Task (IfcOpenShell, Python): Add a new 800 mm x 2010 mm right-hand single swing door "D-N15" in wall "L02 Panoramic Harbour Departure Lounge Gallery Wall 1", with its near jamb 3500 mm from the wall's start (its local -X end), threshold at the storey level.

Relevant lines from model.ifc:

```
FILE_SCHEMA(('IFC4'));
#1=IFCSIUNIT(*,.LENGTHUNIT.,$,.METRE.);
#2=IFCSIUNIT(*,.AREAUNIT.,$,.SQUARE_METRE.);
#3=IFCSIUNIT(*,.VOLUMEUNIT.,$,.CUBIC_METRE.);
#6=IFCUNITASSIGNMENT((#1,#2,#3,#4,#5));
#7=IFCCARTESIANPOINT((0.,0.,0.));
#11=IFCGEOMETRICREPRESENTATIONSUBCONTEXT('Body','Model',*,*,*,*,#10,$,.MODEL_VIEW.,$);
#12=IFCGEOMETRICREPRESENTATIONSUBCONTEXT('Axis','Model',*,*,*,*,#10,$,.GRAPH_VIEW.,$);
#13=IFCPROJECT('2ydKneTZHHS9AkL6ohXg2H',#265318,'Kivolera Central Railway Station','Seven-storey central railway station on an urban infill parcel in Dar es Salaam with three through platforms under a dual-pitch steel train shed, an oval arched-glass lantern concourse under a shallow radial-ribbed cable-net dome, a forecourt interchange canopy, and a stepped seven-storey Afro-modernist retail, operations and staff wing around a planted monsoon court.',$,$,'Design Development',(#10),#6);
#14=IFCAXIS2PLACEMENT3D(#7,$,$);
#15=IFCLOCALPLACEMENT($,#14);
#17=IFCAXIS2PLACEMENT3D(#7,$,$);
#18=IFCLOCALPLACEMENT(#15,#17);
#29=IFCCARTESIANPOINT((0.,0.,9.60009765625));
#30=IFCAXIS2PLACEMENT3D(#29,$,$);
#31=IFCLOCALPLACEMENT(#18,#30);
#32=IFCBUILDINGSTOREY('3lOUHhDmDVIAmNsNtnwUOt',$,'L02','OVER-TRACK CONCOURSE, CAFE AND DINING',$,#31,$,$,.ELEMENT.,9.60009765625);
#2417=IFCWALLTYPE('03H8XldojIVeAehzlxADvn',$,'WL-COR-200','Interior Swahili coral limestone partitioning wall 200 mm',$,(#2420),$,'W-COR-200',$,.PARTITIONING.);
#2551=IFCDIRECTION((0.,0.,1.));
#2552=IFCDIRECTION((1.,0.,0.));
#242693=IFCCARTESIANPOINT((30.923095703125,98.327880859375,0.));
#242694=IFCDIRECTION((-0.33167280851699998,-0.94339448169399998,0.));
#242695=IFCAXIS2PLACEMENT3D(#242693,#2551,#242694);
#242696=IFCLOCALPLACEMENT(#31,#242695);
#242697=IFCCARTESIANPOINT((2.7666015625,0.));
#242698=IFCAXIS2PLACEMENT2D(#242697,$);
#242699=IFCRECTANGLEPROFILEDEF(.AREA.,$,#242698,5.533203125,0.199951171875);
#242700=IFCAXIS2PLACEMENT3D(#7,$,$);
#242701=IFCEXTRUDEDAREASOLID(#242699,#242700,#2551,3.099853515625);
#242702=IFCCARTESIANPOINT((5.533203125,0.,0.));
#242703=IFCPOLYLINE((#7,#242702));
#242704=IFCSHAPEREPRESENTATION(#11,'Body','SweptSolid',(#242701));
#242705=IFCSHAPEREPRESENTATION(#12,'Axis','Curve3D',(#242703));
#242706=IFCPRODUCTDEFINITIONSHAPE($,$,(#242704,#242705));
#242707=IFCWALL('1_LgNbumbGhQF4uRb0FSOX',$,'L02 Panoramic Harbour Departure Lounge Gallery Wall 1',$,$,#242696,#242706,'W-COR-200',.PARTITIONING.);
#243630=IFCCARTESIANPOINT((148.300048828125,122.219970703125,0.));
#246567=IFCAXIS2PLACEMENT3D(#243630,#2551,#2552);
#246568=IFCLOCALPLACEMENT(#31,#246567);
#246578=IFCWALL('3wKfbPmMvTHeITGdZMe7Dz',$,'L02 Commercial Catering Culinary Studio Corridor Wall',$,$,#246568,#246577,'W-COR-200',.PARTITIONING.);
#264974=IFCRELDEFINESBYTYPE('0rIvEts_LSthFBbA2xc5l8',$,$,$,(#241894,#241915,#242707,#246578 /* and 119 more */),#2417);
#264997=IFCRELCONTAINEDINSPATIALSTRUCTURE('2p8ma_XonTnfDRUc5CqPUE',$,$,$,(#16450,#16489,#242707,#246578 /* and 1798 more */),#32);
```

```python
import numpy as np
import ifcopenshell
import ifcopenshell.api.feature
import ifcopenshell.api.geometry
import ifcopenshell.api.root
import ifcopenshell.api.spatial
import ifcopenshell.geom
import ifcopenshell.util.element
import ifcopenshell.util.placement
import ifcopenshell.util.representation
import ifcopenshell.util.shape
import ifcopenshell.util.unit

model = ifcopenshell.open("model.ifc")
unit_scale = ifcopenshell.util.unit.calculate_unit_scale(model)
settings = ifcopenshell.geom.settings()


def volume(element):
    """Net volume in cubic metres, openings subtracted."""
    shape = ifcopenshell.geom.create_shape(settings, element)
    return ifcopenshell.util.shape.get_volume(shape.geometry)


wall = model.by_guid("1_LgNbumbGhQF4uRb0FSOX")
storey = ifcopenshell.util.element.get_container(wall, ifc_class="IfcBuildingStorey")
context = ifcopenshell.util.representation.get_context(model, "Model", "Body", "MODEL_VIEW")
before = volume(wall)

width, height, from_end, sill = 0.8, 2.01, 3.5, 0.0  # metres

# The wall runs along its own X axis, and the end named is its -X end.
wall_shape = ifcopenshell.geom.create_shape(settings, wall)
x, y, z = ifcopenshell.util.shape.get_vertices(wall_shape.geometry).T
start = x.min() + from_end
face, thickness = float(y.min()), float(y.max() - y.min())
wall_matrix = ifcopenshell.util.placement.get_local_placement(wall.ObjectPlacement)
level = ifcopenshell.util.placement.get_local_placement(storey.ObjectPlacement)[2, 3]


def in_wall(x, y):
    """Placement at x, y metres in the wall's axes, at sill height."""
    matrix = wall_matrix.copy()
    matrix[:, 3] = wall_matrix @ np.array([x / unit_scale, y / unit_scale, 0.0, 1.0])
    matrix[2, 3] = level + sill / unit_scale
    return matrix


# Opening: a box that overshoots both wall faces by 50 mm.
opening = ifcopenshell.api.root.create_entity(model, ifc_class="IfcOpeningElement", predefined_type="OPENING")
box = ifcopenshell.api.geometry.add_wall_representation(
    model, context=context, length=width, height=height, thickness=thickness + 0.1
)
ifcopenshell.api.geometry.assign_representation(model, product=opening, representation=box)
ifcopenshell.api.geometry.edit_object_placement(model, product=opening, matrix=in_wall(start, face - 0.05), is_si=False)
ifcopenshell.api.feature.add_feature(model, feature=opening, element=wall)

door = ifcopenshell.api.root.create_entity(model, ifc_class="IfcDoor", name="D-N15", predefined_type="DOOR")
door.OverallWidth, door.OverallHeight = width / unit_scale, height / unit_scale
door.OperationType = "SINGLE_SWING_RIGHT"
body = ifcopenshell.api.geometry.add_door_representation(
    model,
    context=context,
    overall_width=door.OverallWidth,
    overall_height=door.OverallHeight,
    operation_type="SINGLE_SWING_RIGHT",
    lining_properties={"LiningDepth": thickness / unit_scale, "ThresholdDepth": thickness / unit_scale},
)
ifcopenshell.api.geometry.assign_representation(model, product=door, representation=body)
ifcopenshell.api.spatial.assign_container(model, products=[door], relating_structure=storey)
ifcopenshell.api.feature.add_filling(model, opening=opening, element=door)

# The lining spans the wall, so the door starts at the wall face.
ifcopenshell.api.geometry.edit_object_placement(model, product=door, matrix=in_wall(start, face), is_si=False)

after = volume(wall)

print(f"wall volume {before:.3f} -> {after:.3f} m3")

model.write("model_edited.ifc")
```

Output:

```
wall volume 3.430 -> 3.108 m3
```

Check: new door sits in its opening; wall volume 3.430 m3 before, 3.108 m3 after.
